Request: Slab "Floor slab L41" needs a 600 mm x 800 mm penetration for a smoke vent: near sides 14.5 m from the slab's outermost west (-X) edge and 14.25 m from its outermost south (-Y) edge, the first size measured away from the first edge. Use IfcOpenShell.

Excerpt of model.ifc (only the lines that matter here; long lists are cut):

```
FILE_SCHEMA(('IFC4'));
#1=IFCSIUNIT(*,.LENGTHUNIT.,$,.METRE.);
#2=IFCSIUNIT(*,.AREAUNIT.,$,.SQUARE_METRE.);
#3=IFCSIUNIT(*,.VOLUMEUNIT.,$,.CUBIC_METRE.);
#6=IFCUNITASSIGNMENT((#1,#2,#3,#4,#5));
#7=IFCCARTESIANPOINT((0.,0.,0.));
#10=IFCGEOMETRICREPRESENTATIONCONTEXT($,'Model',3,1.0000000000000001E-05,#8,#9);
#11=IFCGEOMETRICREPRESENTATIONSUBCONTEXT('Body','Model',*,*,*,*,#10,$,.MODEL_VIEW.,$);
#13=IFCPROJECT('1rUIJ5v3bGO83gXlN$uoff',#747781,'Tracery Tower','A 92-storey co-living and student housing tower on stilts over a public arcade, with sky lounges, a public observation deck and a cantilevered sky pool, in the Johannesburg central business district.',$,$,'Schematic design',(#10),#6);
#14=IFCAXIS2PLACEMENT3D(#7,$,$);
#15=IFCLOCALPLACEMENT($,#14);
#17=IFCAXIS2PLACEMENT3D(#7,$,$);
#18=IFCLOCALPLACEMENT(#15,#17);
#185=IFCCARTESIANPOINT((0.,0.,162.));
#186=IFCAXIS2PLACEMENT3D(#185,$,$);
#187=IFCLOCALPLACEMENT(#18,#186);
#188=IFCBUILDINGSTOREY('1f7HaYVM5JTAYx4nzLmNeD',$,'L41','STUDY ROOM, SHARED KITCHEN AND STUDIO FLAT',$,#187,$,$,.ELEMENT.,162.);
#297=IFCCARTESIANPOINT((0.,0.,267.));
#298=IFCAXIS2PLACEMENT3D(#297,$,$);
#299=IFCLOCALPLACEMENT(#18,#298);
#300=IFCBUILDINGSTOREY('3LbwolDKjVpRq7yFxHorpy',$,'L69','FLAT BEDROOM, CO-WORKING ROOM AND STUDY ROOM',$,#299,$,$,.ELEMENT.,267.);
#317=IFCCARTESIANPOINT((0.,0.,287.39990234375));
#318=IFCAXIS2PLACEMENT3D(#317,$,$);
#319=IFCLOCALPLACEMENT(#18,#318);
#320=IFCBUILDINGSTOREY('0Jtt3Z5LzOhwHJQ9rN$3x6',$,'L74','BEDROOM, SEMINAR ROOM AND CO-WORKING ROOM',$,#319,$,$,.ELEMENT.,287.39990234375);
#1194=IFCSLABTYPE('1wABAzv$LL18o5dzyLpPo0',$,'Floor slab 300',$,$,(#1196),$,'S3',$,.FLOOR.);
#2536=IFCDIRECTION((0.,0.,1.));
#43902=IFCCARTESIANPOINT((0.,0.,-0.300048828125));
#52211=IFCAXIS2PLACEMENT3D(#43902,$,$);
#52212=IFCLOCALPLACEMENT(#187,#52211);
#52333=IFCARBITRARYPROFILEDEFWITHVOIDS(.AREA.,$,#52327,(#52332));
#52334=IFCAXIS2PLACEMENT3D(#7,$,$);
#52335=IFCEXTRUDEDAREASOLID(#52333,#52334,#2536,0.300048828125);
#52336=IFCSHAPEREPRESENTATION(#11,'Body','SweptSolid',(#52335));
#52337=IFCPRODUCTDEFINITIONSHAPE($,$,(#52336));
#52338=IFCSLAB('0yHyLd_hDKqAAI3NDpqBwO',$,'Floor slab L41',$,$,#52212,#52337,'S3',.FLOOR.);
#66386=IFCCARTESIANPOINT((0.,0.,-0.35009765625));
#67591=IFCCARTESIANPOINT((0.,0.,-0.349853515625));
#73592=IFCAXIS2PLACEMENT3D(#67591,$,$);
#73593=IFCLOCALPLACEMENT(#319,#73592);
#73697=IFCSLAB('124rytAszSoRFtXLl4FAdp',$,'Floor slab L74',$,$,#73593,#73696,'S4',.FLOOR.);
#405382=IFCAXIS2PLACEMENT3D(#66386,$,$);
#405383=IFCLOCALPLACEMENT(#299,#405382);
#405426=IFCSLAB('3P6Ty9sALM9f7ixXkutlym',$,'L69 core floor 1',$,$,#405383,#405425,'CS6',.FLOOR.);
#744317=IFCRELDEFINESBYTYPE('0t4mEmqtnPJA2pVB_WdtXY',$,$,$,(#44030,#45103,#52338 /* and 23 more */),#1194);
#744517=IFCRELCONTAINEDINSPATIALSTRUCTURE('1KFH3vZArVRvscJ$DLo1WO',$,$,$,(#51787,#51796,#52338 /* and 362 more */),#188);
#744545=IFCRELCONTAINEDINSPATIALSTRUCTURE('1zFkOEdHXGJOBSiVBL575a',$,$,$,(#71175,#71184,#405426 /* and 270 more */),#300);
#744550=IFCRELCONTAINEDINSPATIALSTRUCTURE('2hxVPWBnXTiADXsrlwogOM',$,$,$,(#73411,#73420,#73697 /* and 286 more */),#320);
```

```python
import numpy as np
import ifcopenshell
import ifcopenshell.api.feature
import ifcopenshell.api.geometry
import ifcopenshell.api.root
import ifcopenshell.geom
import ifcopenshell.util.placement
import ifcopenshell.util.representation
import ifcopenshell.util.shape
import ifcopenshell.util.unit

model = ifcopenshell.open("model.ifc")
unit_scale = ifcopenshell.util.unit.calculate_unit_scale(model)
settings = ifcopenshell.geom.settings()


def volume(element):
    """Net volume in cubic metres, openings subtracted."""
    shape = ifcopenshell.geom.create_shape(settings, element)
    return ifcopenshell.util.shape.get_volume(shape.geometry)


slab = model.by_guid("0yHyLd_hDKqAAI3NDpqBwO")
before = volume(slab)

# Extent in the slab's own axes, in metres. The edges named are its -X and -Y sides.
slab_shape = ifcopenshell.geom.create_shape(settings, slab)
vertices = ifcopenshell.util.shape.get_vertices(slab_shape.geometry)
x_min, y_min, bottom = vertices.min(axis=0)
top = vertices[:, 2].max()

opening = ifcopenshell.api.root.create_entity(model, ifc_class="IfcOpeningElement", name="Smoke vent opening", predefined_type="OPENING")
context = ifcopenshell.util.representation.get_context(model, "Model", "Body", "MODEL_VIEW")
width, depth = 0.6, 0.8
outline = [(0.0, 0.0), (width, 0.0), (width, depth), (0.0, depth), (0.0, 0.0)]
# Overshoot both faces by 50 mm so the cut is clean.
shape = ifcopenshell.api.geometry.add_slab_representation(
    model, context=context, depth=top - bottom + 0.1, polyline=outline
)
ifcopenshell.api.geometry.assign_representation(model, product=opening, representation=shape)

matrix = ifcopenshell.util.placement.get_local_placement(slab.ObjectPlacement)
matrix[:, 3] = matrix @ np.append(np.array([x_min + 14.5, y_min + 14.25, bottom - 0.05]) / unit_scale, 1.0)
ifcopenshell.api.geometry.edit_object_placement(model, product=opening, matrix=matrix, is_si=False)
ifcopenshell.api.feature.add_feature(model, feature=opening, element=slab)

after = volume(slab)

print(f"slab volume {before:.3f} -> {after:.3f} m3")

model.write("model_edited.ifc")
```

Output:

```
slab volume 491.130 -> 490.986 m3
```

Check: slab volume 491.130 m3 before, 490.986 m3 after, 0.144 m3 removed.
